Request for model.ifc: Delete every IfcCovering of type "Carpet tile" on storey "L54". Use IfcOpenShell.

First a look at what the model holds.

```python
import ifcopenshell
import ifcopenshell.util.element

model = ifcopenshell.open("model.ifc")
print(model.schema)
storey = next(s for s in model.by_type("IfcBuildingStorey") if s.Name == "L54")
coverings = [e for e in ifcopenshell.util.element.get_decomposition(storey) if e.is_a("IfcCovering")]
seen = {}
for e in coverings:
    element_type = ifcopenshell.util.element.get_type(e)
    name = element_type.Name if element_type not in (None, e) else None
    seen[name] = seen.get(name, 0) + 1
for name, count in sorted(seen.items(), key=str):
    print(count, "x", name)
```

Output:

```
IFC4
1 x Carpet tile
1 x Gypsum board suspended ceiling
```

```python
import ifcopenshell
import ifcopenshell.api.root
import ifcopenshell.util.element

model = ifcopenshell.open("model.ifc")

storey = next(s for s in model.by_type("IfcBuildingStorey") if s.Name == "L54")
coverings = [e for e in ifcopenshell.util.element.get_decomposition(storey) if e.is_a("IfcCovering")]
targets = [e for e in coverings if (t := ifcopenshell.util.element.get_type(e)) not in (None, e) and t.Name == "Carpet tile"]

for e in targets:
    ifcopenshell.api.root.remove_product(model, product=e)
print(len(targets), "removed")

model.write("model_edited.ifc")
```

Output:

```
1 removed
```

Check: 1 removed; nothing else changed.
